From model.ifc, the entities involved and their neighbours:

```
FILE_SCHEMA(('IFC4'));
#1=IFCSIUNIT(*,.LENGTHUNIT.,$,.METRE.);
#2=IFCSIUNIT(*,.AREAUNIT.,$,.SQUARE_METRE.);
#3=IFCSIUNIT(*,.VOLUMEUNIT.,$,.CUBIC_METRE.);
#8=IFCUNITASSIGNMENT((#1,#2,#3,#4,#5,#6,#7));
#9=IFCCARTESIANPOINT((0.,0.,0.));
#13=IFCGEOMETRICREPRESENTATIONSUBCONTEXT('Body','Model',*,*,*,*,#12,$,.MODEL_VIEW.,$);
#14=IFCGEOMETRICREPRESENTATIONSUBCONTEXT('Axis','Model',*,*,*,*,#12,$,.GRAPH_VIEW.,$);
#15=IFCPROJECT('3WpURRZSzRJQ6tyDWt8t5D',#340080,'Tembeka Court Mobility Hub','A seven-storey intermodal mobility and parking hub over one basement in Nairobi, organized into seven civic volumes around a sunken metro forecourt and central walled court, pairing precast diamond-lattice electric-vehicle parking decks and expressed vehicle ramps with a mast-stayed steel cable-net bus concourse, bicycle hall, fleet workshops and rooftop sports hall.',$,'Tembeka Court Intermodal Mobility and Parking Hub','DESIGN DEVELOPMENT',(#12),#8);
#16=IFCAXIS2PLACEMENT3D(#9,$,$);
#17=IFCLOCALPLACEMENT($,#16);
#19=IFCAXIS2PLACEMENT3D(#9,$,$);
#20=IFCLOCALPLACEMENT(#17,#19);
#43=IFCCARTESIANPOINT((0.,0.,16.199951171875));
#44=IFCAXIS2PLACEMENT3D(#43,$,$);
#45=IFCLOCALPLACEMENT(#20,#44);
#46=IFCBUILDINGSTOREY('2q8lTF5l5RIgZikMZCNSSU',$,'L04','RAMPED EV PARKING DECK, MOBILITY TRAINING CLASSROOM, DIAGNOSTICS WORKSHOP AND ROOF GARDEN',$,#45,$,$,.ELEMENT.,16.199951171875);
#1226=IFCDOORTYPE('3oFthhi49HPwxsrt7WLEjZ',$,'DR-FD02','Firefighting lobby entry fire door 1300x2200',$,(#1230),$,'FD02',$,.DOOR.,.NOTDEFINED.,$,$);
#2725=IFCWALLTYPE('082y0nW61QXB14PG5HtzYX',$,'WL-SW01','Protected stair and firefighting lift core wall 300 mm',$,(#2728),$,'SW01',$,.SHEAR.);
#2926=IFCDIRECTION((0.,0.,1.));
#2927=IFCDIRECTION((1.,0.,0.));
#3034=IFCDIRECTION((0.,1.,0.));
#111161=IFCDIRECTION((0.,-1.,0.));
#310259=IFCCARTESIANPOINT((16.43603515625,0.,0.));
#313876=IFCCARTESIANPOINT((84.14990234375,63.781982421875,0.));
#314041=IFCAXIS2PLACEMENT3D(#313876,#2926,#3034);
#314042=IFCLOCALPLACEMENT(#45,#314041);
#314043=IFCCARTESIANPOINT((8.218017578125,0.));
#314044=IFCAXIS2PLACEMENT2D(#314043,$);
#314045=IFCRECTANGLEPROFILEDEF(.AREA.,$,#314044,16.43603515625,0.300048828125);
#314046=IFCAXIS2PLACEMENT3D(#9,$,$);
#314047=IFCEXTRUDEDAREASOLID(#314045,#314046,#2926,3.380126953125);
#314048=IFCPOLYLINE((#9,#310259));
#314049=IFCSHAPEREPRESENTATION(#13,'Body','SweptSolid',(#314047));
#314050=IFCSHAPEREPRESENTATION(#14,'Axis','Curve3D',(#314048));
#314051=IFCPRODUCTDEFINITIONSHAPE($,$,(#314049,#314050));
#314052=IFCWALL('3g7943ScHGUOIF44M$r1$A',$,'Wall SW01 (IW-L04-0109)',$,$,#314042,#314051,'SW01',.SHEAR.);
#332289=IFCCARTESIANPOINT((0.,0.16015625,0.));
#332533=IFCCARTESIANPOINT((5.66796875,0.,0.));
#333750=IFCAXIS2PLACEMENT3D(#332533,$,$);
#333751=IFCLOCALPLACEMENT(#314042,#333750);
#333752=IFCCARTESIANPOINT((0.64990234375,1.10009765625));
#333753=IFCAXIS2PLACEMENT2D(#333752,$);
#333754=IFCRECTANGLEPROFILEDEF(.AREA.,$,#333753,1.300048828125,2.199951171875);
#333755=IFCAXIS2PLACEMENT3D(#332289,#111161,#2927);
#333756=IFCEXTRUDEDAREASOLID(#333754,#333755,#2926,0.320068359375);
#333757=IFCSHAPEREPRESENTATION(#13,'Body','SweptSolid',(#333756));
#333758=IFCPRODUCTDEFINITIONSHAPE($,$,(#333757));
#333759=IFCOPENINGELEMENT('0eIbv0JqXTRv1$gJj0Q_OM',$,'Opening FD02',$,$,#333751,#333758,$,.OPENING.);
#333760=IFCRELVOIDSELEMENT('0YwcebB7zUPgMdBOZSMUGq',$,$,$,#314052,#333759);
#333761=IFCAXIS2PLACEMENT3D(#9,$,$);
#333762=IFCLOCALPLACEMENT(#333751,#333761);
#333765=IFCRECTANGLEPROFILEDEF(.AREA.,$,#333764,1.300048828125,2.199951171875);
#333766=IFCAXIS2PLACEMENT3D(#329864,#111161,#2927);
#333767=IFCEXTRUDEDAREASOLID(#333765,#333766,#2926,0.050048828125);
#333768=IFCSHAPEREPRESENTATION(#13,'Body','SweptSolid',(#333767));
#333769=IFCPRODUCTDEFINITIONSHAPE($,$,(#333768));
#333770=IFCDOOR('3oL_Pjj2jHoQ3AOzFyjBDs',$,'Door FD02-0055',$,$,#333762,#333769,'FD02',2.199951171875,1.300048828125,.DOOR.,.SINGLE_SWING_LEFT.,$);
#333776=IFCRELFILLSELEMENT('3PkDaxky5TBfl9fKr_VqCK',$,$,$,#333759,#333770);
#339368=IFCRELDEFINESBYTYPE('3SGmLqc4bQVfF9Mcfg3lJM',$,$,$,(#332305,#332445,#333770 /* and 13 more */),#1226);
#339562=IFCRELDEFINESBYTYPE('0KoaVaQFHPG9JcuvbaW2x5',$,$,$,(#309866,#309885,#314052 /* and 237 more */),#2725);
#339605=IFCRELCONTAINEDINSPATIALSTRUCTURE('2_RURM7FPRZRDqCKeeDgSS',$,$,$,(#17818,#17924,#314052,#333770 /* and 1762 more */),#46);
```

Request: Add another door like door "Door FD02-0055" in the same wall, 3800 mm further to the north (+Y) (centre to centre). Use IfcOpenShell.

```python
import ifcopenshell
import ifcopenshell.api.feature
import ifcopenshell.api.geometry
import ifcopenshell.api.root
import ifcopenshell.geom
import ifcopenshell.util.element
import ifcopenshell.util.placement
import ifcopenshell.util.shape

model = ifcopenshell.open("model.ifc")
settings = ifcopenshell.geom.settings()


def volume(element):
    """Net volume in cubic metres, openings subtracted."""
    shape = ifcopenshell.geom.create_shape(settings, element)
    return ifcopenshell.util.shape.get_volume(shape.geometry)


door = model.by_id(333770)
opening = door.FillsVoids[0].RelatingOpeningElement
wall = opening.VoidsElements[0].RelatingBuildingElement
before = volume(wall)
shift = ifcopenshell.util.placement.get_local_placement(wall.ObjectPlacement)[:3, 0] * 3.8

# copy_class copies the void relationship, type, container and properties, but no geometry.
new_opening = ifcopenshell.api.root.copy_class(model, product=opening)
new_opening.Representation = ifcopenshell.util.element.copy_deep(
    model, opening.Representation, exclude=["IfcGeometricRepresentationContext", "IfcRepresentationMap"]
)
new_door = ifcopenshell.api.root.copy_class(model, product=door)
new_door.Representation = ifcopenshell.util.element.copy_deep(
    model, door.Representation, exclude=["IfcGeometricRepresentationContext", "IfcRepresentationMap"]
)
new_door.Tag = None
ifcopenshell.api.feature.add_filling(model, opening=new_opening, element=new_door)

for old, new in ((opening, new_opening), (door, new_door)):
    matrix = ifcopenshell.util.placement.get_local_placement(old.ObjectPlacement)
    matrix[:3, 3] += shift
    ifcopenshell.api.geometry.edit_object_placement(model, product=new, matrix=matrix, is_si=False)

after = volume(wall)

print(f"wall volume {before:.3f} -> {after:.3f} m3")

model.write("model_edited.ifc")
```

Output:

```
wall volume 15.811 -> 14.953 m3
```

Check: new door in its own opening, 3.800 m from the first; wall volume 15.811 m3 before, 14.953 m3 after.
